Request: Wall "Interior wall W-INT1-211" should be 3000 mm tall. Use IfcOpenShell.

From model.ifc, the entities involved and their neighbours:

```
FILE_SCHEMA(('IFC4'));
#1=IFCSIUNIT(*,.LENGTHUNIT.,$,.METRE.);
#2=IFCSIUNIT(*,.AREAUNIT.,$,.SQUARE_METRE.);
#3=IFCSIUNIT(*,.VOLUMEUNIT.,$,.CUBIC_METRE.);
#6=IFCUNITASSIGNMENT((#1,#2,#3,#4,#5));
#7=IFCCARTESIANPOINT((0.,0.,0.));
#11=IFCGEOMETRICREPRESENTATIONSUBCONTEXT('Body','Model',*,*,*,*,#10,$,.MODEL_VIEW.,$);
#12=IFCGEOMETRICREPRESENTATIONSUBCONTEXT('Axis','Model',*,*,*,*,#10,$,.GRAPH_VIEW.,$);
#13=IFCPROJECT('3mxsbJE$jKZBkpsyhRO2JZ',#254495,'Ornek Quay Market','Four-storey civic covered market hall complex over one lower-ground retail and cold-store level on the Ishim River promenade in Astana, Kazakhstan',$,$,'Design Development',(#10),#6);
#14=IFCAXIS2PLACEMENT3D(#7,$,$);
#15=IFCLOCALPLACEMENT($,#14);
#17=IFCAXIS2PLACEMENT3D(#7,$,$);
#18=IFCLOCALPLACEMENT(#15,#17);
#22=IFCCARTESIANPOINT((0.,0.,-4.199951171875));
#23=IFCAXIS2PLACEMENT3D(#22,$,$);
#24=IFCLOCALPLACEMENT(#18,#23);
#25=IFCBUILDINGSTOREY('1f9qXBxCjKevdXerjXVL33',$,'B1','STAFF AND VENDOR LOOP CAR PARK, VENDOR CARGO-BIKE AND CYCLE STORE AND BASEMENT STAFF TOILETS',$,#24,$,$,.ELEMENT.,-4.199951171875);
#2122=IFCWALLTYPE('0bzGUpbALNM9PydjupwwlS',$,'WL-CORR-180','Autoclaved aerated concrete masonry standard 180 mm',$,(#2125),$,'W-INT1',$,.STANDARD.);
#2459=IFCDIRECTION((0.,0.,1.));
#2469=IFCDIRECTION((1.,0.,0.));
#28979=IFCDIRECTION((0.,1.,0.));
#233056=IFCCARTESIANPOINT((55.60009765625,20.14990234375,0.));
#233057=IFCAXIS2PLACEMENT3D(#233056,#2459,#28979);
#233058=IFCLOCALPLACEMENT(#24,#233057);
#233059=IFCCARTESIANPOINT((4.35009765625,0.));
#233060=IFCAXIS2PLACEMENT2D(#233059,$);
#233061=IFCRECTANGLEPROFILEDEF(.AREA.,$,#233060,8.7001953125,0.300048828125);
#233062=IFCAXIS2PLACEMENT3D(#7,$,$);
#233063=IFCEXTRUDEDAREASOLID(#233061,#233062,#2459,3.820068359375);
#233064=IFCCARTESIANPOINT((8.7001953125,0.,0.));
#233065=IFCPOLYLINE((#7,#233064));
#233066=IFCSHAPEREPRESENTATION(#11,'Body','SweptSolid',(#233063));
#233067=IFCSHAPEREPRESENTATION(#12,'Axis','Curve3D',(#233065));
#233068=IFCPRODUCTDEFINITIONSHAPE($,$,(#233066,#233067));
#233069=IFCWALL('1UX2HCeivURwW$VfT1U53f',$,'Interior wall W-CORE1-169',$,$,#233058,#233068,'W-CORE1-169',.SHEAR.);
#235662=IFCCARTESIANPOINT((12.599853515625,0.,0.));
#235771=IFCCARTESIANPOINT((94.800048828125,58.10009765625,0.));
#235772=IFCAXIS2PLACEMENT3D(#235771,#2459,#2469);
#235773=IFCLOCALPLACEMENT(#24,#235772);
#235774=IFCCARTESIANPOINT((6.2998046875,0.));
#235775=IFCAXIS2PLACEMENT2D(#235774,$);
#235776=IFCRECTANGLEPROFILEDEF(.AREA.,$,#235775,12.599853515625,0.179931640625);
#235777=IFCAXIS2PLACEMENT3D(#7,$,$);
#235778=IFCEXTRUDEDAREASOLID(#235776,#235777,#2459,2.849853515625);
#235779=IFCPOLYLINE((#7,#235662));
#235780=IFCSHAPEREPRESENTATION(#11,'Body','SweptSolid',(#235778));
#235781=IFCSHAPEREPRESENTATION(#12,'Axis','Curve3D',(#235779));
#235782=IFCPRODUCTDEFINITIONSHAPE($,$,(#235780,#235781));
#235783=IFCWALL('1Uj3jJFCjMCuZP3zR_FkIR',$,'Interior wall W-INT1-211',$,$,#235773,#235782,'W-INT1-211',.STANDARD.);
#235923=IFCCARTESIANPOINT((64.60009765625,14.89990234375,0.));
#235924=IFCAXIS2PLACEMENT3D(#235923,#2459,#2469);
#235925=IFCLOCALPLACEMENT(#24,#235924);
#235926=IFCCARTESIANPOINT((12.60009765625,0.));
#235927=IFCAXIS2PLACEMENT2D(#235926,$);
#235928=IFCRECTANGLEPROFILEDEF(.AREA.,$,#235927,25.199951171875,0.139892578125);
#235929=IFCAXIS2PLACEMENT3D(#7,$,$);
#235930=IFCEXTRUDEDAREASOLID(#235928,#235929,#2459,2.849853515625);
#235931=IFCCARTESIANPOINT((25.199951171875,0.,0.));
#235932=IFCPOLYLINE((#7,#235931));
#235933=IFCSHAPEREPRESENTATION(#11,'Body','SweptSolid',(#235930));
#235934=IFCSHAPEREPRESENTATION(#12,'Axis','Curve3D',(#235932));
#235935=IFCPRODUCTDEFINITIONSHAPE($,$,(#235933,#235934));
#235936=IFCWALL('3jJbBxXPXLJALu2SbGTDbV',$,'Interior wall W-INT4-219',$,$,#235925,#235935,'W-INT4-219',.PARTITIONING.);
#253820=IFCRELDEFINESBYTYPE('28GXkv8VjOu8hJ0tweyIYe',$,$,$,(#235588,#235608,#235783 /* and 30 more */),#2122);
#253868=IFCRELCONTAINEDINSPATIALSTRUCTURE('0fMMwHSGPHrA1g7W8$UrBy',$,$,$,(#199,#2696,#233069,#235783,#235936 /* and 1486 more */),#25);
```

```python
import ifcopenshell
import ifcopenshell.geom
import ifcopenshell.util.representation
import ifcopenshell.util.shape
import ifcopenshell.util.unit

model = ifcopenshell.open("model.ifc")
unit_scale = ifcopenshell.util.unit.calculate_unit_scale(model)
settings = ifcopenshell.geom.settings()


def volume(element):
    """Net volume in cubic metres, openings subtracted."""
    shape = ifcopenshell.geom.create_shape(settings, element)
    return ifcopenshell.util.shape.get_volume(shape.geometry)


wall = model.by_guid("1Uj3jJFCjMCuZP3zR_FkIR")
before = volume(wall)

body = ifcopenshell.util.representation.get_representation(wall, "Model", "Body")
solid = body.Items[0]
old_height = solid.Depth
solid.Depth = 3 / unit_scale
after = volume(wall)

print(f"height {old_height:g} -> {solid.Depth:g}, volume {before:.3f} -> {after:.3f} m3")

model.write("model_updated.ifc")
```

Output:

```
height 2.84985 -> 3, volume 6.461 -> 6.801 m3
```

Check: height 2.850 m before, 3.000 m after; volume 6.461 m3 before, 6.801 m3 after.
